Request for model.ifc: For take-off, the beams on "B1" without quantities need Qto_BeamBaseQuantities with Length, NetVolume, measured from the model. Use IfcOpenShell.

First a look at what the model holds.

```python
import ifcopenshell
import ifcopenshell.util.element
import ifcopenshell.util.unit

model = ifcopenshell.open("model.ifc")
print(model.schema)
for unit_type in ("LENGTHUNIT", "AREAUNIT", "VOLUMEUNIT"):
    print(unit_type, ifcopenshell.util.unit.calculate_unit_scale(model, unit_type))
storey = next(s for s in model.by_type("IfcBuildingStorey") if s.Name == "B1")
beams = [e for e in ifcopenshell.util.element.get_decomposition(storey) if e.is_a("IfcBeam")]
for e in sorted(beams, key=lambda e: e.id()):
    print(e.id(), e.is_a(), e.Name, list(ifcopenshell.util.element.get_psets(e, qtos_only=True)), sep=" | ")
```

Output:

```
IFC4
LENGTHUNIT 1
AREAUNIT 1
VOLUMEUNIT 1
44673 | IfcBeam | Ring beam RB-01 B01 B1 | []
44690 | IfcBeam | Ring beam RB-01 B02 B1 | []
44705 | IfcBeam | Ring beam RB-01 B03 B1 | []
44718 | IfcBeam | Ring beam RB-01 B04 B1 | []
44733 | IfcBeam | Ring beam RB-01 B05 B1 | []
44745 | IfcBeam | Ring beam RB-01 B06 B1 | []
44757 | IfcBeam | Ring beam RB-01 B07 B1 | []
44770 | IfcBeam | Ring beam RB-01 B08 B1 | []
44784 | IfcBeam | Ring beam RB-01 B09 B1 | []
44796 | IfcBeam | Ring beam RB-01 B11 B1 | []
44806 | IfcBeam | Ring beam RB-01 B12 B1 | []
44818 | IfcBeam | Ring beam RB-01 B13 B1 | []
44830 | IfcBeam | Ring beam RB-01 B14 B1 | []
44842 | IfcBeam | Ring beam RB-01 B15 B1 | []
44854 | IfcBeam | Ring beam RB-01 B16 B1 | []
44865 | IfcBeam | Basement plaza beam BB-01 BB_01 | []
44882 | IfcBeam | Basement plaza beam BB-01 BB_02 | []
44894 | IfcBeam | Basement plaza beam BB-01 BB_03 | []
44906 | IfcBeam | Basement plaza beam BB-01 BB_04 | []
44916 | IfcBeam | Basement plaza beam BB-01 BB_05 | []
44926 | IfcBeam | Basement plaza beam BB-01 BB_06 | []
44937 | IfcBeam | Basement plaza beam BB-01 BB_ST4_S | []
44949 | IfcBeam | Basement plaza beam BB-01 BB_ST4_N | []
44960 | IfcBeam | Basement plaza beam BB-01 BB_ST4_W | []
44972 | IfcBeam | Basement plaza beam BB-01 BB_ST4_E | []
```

```python
import ifcopenshell
import ifcopenshell.api.pset
import ifcopenshell.geom
import ifcopenshell.util.element
import ifcopenshell.util.shape
import ifcopenshell.util.unit

model = ifcopenshell.open("model.ifc")
unit_scale = ifcopenshell.util.unit.calculate_unit_scale(model)
volume_scale = ifcopenshell.util.unit.calculate_unit_scale(model, "VOLUMEUNIT")
settings = ifcopenshell.geom.settings()

storey = next(s for s in model.by_type("IfcBuildingStorey") if s.Name == "B1")
beams = [e for e in ifcopenshell.util.element.get_decomposition(storey) if e.is_a("IfcBeam")]

for e in sorted(beams, key=lambda e: e.id()):
    if ifcopenshell.util.element.get_psets(e, qtos_only=True, should_inherit=False):
        continue
    # Geometry comes back in metres, in the element's own axes.
    shape = ifcopenshell.geom.create_shape(settings, e)
    values = {
        "Length": ifcopenshell.util.shape.get_max_xyz(shape.geometry) / unit_scale,
        "NetVolume": ifcopenshell.util.shape.get_volume(shape.geometry) / volume_scale,
    }
    qto = ifcopenshell.api.pset.add_qto(model, product=e, name="Qto_BeamBaseQuantities")
    ifcopenshell.api.pset.edit_qto(model, qto=qto, properties=values)
    print(e.id(), {k: round(v, 3) for k, v in values.items()})

model.write("model_edited.ifc")
```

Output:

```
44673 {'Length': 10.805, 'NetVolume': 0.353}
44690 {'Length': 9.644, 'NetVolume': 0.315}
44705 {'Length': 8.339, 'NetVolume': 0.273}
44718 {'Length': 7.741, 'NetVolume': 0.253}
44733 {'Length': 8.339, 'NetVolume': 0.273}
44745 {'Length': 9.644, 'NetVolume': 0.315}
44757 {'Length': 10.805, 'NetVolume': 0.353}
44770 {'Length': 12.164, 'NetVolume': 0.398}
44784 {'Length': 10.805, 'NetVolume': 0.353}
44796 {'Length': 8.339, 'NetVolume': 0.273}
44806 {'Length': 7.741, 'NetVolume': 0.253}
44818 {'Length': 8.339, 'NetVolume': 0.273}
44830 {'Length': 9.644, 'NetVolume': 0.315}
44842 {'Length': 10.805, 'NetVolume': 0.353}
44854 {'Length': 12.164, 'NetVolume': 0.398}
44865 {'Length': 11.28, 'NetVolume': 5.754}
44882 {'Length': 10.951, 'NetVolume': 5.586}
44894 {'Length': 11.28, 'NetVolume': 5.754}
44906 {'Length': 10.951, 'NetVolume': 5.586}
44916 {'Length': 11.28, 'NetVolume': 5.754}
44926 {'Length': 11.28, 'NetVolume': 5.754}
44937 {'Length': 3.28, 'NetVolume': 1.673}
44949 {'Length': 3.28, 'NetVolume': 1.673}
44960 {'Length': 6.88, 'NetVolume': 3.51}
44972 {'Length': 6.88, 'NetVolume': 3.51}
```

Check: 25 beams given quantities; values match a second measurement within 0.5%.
